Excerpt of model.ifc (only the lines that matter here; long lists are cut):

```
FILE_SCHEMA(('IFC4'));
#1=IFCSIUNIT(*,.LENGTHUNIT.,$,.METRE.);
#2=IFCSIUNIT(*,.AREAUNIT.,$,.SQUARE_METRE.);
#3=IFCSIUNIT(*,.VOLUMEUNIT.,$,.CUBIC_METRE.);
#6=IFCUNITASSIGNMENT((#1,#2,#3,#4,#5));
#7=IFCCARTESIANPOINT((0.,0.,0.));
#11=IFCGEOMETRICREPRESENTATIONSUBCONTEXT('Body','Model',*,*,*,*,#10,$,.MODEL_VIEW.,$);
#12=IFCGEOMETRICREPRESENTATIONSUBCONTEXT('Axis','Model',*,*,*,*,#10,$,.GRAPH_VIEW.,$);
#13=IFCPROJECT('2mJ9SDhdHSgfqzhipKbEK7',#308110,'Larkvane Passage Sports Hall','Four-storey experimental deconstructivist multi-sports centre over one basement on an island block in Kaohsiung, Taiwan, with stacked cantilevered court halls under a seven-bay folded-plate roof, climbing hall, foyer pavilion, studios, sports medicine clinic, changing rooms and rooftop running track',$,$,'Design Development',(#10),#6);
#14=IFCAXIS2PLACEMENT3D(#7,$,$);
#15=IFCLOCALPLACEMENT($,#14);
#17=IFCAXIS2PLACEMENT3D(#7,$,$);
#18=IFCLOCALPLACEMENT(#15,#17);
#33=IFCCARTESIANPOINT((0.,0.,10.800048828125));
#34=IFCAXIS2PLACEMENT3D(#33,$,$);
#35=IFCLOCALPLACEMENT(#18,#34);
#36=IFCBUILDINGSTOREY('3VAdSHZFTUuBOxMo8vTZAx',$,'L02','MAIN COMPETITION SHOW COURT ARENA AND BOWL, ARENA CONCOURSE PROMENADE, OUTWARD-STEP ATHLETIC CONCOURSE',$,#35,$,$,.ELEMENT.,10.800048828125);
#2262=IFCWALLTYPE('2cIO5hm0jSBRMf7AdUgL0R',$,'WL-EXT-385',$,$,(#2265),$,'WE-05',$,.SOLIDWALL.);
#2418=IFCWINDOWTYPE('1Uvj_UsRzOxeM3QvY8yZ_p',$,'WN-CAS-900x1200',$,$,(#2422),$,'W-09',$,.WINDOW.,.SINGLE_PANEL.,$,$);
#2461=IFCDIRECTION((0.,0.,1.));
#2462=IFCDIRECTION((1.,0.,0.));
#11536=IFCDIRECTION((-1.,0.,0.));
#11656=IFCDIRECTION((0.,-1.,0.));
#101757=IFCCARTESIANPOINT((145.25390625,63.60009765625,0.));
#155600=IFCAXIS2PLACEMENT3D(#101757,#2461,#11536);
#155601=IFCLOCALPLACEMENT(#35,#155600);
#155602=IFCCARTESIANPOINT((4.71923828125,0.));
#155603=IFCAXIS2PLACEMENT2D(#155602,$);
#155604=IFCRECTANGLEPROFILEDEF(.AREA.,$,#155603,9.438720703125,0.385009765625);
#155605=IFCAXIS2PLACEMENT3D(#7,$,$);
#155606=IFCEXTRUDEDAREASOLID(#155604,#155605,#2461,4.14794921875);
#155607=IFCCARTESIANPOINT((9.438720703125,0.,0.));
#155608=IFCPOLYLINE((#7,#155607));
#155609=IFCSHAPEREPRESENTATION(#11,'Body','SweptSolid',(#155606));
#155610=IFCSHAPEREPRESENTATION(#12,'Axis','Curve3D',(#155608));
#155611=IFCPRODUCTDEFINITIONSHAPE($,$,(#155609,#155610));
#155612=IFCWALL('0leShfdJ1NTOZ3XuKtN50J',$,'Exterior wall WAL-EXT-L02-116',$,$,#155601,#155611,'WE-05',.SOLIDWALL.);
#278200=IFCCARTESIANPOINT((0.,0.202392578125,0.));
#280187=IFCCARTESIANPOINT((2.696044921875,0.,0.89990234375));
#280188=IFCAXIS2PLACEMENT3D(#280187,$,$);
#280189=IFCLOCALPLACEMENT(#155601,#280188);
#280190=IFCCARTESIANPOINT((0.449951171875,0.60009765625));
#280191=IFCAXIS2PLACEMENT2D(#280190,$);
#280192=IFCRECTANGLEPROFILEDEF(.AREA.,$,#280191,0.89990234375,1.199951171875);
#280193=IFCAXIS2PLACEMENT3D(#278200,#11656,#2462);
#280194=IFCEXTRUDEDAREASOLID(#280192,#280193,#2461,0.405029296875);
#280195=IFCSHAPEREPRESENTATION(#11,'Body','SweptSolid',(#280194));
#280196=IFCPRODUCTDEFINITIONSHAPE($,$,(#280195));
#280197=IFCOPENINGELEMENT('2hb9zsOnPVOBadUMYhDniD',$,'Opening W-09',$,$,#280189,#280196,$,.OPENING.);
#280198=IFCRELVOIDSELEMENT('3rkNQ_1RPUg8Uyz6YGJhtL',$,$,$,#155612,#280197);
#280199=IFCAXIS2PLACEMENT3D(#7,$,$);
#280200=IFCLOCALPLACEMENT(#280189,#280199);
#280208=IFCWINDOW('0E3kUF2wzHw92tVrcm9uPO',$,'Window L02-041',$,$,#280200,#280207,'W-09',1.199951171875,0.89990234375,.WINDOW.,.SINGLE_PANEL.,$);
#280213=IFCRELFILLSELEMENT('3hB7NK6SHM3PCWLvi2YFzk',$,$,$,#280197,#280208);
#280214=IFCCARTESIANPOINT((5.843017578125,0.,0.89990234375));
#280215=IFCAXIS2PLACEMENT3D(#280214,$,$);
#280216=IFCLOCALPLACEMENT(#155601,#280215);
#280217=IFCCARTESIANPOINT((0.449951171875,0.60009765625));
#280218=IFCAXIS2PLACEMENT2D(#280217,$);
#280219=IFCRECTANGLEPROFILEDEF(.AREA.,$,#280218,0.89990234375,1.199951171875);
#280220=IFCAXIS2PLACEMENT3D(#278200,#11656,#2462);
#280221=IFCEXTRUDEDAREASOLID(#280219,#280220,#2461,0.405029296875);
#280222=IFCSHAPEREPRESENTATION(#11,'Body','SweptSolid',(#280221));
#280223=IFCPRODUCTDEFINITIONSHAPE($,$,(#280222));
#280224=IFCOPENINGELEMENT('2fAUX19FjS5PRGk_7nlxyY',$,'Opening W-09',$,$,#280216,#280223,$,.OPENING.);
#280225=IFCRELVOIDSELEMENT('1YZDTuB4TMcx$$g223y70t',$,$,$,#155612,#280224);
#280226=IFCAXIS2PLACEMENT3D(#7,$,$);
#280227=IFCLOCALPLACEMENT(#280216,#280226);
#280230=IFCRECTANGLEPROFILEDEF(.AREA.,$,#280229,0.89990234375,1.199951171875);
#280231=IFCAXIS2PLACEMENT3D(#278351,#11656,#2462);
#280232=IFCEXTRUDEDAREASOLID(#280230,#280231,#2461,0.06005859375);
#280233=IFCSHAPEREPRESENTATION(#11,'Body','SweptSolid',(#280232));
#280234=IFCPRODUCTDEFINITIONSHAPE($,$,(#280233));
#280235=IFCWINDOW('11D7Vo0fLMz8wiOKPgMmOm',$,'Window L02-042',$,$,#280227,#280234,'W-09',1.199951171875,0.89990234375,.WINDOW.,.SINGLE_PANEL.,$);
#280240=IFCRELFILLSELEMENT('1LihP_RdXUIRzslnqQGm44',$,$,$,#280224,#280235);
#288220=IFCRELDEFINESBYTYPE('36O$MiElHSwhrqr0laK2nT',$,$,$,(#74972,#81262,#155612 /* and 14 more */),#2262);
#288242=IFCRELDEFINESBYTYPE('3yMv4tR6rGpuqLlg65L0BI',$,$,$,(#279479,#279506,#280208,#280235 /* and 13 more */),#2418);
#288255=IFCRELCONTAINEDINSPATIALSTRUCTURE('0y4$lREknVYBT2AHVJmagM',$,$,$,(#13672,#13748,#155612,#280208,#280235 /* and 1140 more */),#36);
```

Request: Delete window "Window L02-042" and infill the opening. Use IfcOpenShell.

```python
import ifcopenshell
import ifcopenshell.api.feature
import ifcopenshell.api.root
import ifcopenshell.geom
import ifcopenshell.util.shape

model = ifcopenshell.open("model.ifc")
settings = ifcopenshell.geom.settings()


def volume(element):
    """Net volume in cubic metres, openings subtracted."""
    shape = ifcopenshell.geom.create_shape(settings, element)
    return ifcopenshell.util.shape.get_volume(shape.geometry)


window = model.by_guid("11D7Vo0fLMz8wiOKPgMmOm")
opening = window.FillsVoids[0].RelatingOpeningElement
wall = opening.VoidsElements[0].RelatingBuildingElement
before = volume(wall)

ifcopenshell.api.root.remove_product(model, product=window)
ifcopenshell.api.feature.remove_feature(model, feature=opening)

after = volume(wall)

print(f"wall volume {before:.3f} -> {after:.3f} m3")

model.write("model-out.ifc")
```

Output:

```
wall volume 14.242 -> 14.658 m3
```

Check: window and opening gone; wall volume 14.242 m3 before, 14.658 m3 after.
